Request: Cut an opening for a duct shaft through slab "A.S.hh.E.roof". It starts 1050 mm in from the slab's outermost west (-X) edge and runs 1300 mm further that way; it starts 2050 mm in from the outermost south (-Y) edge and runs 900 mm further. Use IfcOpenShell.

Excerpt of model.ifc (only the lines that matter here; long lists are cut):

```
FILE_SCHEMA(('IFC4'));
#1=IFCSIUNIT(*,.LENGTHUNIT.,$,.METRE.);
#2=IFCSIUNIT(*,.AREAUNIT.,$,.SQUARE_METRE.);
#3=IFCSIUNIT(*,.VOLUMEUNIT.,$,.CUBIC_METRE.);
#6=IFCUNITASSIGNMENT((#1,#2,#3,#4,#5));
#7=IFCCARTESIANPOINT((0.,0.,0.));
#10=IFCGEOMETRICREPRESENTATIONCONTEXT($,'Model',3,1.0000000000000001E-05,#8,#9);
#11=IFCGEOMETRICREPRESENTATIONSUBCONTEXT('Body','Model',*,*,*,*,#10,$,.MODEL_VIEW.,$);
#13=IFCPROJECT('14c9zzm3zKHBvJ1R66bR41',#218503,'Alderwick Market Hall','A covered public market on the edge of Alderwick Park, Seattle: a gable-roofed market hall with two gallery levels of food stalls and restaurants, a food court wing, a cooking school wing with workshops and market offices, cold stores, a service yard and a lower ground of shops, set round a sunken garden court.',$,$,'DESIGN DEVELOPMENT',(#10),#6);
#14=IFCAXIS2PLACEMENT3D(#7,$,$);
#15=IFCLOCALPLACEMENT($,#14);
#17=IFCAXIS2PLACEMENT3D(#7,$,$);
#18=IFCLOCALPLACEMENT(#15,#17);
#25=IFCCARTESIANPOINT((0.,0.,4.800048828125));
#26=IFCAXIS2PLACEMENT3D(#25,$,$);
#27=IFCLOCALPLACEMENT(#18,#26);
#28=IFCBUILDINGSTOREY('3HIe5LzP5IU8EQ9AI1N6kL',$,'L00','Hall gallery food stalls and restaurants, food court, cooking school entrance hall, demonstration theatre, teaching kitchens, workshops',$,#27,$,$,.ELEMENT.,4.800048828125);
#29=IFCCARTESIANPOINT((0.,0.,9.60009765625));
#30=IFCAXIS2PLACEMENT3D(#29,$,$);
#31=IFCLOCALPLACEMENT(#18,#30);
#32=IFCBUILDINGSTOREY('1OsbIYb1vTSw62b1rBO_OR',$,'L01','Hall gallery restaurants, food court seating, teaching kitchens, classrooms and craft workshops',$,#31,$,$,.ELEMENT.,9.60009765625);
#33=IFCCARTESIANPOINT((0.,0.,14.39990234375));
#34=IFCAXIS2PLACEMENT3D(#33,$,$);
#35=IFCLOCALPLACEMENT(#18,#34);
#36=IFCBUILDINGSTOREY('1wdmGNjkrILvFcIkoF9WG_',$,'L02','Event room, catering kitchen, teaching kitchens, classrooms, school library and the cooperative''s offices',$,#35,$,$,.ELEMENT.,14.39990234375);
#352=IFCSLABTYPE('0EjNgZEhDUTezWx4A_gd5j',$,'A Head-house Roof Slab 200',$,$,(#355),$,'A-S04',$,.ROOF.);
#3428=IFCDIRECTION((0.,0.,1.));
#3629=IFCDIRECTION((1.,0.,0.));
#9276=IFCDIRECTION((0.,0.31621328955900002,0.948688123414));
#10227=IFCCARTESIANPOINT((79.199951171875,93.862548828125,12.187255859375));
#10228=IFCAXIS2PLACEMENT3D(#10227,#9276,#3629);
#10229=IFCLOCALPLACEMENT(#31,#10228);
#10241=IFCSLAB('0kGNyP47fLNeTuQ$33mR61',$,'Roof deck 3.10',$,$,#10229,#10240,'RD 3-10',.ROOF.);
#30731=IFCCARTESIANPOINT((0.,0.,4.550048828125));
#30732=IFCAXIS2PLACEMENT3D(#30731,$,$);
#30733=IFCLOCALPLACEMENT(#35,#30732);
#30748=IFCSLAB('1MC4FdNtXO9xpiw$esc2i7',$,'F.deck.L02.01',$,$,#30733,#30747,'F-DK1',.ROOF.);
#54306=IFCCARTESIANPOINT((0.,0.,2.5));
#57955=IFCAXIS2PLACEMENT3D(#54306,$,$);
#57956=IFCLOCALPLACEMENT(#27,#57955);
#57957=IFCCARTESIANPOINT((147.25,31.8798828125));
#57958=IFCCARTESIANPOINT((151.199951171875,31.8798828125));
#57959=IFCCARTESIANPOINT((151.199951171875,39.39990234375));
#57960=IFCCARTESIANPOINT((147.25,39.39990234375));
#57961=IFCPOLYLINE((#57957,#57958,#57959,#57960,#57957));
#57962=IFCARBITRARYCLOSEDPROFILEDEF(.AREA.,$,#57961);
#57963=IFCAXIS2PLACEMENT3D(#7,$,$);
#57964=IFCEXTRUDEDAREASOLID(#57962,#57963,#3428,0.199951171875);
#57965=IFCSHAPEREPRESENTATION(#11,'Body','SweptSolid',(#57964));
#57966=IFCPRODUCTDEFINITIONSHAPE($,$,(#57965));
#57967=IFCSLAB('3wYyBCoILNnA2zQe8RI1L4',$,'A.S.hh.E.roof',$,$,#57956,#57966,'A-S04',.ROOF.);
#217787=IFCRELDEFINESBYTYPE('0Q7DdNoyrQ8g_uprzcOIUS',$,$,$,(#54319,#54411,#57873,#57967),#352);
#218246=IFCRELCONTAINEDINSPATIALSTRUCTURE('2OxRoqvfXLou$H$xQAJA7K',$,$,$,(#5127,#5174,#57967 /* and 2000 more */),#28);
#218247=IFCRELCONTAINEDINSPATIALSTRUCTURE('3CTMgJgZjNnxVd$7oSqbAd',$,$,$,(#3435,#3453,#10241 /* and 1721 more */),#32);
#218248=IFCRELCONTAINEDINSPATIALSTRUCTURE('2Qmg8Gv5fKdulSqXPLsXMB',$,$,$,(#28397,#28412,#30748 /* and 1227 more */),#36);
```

```python
import numpy as np
import ifcopenshell
import ifcopenshell.api.feature
import ifcopenshell.api.geometry
import ifcopenshell.api.root
import ifcopenshell.geom
import ifcopenshell.util.placement
import ifcopenshell.util.representation
import ifcopenshell.util.shape
import ifcopenshell.util.unit

model = ifcopenshell.open("model.ifc")
unit_scale = ifcopenshell.util.unit.calculate_unit_scale(model)
settings = ifcopenshell.geom.settings()


def volume(element):
    """Net volume in cubic metres, openings subtracted."""
    shape = ifcopenshell.geom.create_shape(settings, element)
    return ifcopenshell.util.shape.get_volume(shape.geometry)


slab = model.by_guid("3wYyBCoILNnA2zQe8RI1L4")
before = volume(slab)

# Extent in the slab's own axes, in metres. The edges named are its -X and -Y sides.
slab_shape = ifcopenshell.geom.create_shape(settings, slab)
vertices = ifcopenshell.util.shape.get_vertices(slab_shape.geometry)
x_min, y_min, bottom = vertices.min(axis=0)
top = vertices[:, 2].max()

opening = ifcopenshell.api.root.create_entity(model, ifc_class="IfcOpeningElement", name="Duct shaft opening", predefined_type="OPENING")
context = ifcopenshell.util.representation.get_context(model, "Model", "Body", "MODEL_VIEW")
width, depth = 1.3, 0.9
outline = [(0.0, 0.0), (width, 0.0), (width, depth), (0.0, depth), (0.0, 0.0)]
# Overshoot both faces by 50 mm so the cut is clean.
shape = ifcopenshell.api.geometry.add_slab_representation(
    model, context=context, depth=top - bottom + 0.1, polyline=outline
)
ifcopenshell.api.geometry.assign_representation(model, product=opening, representation=shape)

matrix = ifcopenshell.util.placement.get_local_placement(slab.ObjectPlacement)
matrix[:, 3] = matrix @ np.append(np.array([x_min + 1.05, y_min + 2.05, bottom - 0.05]) / unit_scale, 1.0)
ifcopenshell.api.geometry.edit_object_placement(model, product=opening, matrix=matrix, is_si=False)
ifcopenshell.api.feature.add_feature(model, feature=opening, element=slab)

after = volume(slab)

print(f"slab volume {before:.3f} -> {after:.3f} m3")

model.write("model_edited.ifc")
```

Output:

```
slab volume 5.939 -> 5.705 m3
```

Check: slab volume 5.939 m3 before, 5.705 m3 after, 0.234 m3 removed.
